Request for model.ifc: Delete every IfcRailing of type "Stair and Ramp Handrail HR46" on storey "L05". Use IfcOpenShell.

First a look at what the model holds.

```python
import ifcopenshell
import ifcopenshell.util.element

model = ifcopenshell.open("model.ifc")
print(model.schema)
storey = next(s for s in model.by_type("IfcBuildingStorey") if s.Name == "L05")
railings = [e for e in ifcopenshell.util.element.get_decomposition(storey) if e.is_a("IfcRailing")]
seen = {}
for e in railings:
    element_type = ifcopenshell.util.element.get_type(e)
    name = element_type.Name if element_type not in (None, e) else None
    seen[name] = seen.get(name, 0) + 1
for name, count in sorted(seen.items(), key=str):
    print(count, "x", name)
```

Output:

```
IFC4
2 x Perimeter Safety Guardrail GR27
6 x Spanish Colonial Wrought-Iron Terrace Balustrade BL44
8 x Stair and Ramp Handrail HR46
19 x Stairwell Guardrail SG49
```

```python
import ifcopenshell
import ifcopenshell.api.root
import ifcopenshell.util.element

model = ifcopenshell.open("model.ifc")

storey = next(s for s in model.by_type("IfcBuildingStorey") if s.Name == "L05")
railings = [e for e in ifcopenshell.util.element.get_decomposition(storey) if e.is_a("IfcRailing")]
targets = [e for e in railings if (t := ifcopenshell.util.element.get_type(e)) not in (None, e) and t.Name == "Stair and Ramp Handrail HR46"]

for e in targets:
    ifcopenshell.api.root.remove_product(model, product=e)
print(len(targets), "removed")

model.write("model-out.ifc")
```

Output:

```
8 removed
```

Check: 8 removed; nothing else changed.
